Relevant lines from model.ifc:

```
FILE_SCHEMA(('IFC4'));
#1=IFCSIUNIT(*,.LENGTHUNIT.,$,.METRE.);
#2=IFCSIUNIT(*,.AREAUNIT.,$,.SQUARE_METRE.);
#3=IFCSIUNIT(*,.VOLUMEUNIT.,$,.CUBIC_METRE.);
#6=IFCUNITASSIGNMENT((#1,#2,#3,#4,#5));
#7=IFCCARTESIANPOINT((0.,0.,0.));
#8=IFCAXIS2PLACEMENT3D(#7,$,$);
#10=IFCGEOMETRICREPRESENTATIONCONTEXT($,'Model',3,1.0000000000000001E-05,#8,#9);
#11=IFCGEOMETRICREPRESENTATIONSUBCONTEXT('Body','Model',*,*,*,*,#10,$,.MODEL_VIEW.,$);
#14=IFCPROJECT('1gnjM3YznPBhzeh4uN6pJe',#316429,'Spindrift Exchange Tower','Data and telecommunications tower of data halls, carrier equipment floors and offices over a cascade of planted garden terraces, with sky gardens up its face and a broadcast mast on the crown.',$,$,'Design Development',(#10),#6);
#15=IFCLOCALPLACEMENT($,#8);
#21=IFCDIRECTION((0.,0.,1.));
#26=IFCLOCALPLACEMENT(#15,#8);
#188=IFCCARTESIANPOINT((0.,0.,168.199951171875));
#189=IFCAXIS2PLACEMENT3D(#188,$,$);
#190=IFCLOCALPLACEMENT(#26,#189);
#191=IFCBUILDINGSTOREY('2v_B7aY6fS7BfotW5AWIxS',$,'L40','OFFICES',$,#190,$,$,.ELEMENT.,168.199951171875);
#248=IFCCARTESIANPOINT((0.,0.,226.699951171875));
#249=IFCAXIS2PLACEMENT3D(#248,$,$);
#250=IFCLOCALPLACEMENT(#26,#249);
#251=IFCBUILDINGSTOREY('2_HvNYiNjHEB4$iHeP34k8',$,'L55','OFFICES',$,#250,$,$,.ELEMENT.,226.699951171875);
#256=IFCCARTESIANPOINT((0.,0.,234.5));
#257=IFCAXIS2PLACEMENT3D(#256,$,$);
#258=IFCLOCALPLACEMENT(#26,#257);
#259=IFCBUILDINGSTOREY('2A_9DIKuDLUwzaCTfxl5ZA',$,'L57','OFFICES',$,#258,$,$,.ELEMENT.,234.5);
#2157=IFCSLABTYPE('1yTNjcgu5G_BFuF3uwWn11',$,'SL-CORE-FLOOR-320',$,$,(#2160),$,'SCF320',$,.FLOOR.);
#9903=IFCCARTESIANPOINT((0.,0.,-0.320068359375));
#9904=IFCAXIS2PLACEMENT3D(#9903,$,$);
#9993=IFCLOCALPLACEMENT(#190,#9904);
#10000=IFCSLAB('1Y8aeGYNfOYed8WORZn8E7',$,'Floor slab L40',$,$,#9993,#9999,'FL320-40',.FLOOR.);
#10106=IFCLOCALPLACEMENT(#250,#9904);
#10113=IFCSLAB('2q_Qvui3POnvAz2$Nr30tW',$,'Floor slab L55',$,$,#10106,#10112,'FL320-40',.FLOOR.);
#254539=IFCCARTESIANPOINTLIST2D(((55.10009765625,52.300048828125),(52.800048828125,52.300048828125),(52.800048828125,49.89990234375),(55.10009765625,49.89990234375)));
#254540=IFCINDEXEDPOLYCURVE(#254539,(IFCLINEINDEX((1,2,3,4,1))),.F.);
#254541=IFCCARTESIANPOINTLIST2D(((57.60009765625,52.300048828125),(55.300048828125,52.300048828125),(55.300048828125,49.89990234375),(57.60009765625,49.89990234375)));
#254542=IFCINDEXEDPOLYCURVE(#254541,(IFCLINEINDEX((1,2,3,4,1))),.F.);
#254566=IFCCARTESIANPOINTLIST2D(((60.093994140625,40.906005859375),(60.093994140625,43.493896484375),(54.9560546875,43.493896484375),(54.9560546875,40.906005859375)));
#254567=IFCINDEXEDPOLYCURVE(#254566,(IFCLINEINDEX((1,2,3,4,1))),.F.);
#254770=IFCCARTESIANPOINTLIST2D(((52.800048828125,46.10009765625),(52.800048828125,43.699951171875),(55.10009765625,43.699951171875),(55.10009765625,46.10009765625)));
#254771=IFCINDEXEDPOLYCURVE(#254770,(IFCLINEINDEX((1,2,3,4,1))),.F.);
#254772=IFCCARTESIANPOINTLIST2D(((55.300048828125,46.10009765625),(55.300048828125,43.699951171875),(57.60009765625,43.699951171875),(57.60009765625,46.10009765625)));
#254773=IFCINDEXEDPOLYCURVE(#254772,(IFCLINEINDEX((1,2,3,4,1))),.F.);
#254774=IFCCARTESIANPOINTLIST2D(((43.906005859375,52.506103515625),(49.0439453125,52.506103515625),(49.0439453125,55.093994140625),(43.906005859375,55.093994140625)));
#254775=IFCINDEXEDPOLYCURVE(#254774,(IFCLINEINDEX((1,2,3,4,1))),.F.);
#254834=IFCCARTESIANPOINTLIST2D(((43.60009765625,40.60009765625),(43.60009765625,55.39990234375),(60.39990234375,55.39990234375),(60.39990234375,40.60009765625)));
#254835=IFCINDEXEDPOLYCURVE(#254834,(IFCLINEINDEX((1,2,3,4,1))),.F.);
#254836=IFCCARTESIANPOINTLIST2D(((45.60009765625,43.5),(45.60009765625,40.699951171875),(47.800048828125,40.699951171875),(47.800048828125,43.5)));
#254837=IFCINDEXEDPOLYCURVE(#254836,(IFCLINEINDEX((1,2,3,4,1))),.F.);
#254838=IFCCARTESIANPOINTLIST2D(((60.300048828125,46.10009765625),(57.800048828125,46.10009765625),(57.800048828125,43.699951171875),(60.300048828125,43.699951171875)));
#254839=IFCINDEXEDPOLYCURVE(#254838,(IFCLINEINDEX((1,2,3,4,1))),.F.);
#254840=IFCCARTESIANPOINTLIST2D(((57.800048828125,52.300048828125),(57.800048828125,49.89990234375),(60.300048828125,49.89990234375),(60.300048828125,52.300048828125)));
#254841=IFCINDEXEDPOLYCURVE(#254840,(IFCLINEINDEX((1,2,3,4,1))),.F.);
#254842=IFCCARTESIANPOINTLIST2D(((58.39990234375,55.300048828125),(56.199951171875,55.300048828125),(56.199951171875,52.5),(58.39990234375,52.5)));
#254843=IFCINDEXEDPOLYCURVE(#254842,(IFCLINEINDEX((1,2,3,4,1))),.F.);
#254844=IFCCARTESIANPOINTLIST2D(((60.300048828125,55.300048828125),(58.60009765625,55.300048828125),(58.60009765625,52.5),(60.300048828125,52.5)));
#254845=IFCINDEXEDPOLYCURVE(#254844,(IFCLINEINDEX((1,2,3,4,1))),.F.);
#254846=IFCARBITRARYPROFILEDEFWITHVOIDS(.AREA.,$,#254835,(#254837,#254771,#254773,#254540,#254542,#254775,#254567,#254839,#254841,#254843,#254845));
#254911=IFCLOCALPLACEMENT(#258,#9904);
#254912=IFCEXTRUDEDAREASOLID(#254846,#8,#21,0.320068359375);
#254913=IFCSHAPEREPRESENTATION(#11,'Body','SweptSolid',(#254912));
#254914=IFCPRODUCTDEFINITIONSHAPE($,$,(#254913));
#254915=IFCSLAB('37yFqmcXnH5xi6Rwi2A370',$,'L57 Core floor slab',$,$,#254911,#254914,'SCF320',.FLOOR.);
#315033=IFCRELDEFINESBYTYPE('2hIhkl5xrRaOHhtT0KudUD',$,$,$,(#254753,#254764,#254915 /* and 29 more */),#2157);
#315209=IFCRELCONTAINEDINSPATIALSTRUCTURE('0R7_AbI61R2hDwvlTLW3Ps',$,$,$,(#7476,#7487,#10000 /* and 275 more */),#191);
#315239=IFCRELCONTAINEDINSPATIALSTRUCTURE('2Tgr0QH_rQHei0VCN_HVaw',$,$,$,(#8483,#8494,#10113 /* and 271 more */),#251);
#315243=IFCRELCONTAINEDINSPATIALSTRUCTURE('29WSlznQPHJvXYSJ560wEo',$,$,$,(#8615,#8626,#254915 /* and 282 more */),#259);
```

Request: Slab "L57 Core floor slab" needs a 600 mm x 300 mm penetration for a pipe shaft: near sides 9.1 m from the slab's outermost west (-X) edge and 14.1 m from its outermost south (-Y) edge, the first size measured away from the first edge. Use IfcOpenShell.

```python
import numpy as np
import ifcopenshell
import ifcopenshell.api.feature
import ifcopenshell.api.geometry
import ifcopenshell.api.root
import ifcopenshell.geom
import ifcopenshell.util.placement
import ifcopenshell.util.representation
import ifcopenshell.util.shape
import ifcopenshell.util.unit

model = ifcopenshell.open("model.ifc")
unit_scale = ifcopenshell.util.unit.calculate_unit_scale(model)
settings = ifcopenshell.geom.settings()


def volume(element):
    """Net volume in cubic metres, openings subtracted."""
    shape = ifcopenshell.geom.create_shape(settings, element)
    return ifcopenshell.util.shape.get_volume(shape.geometry)


slab = model.by_guid("37yFqmcXnH5xi6Rwi2A370")
before = volume(slab)

# Extent in the slab's own axes, in metres. The edges named are its -X and -Y sides.
slab_shape = ifcopenshell.geom.create_shape(settings, slab)
vertices = ifcopenshell.util.shape.get_vertices(slab_shape.geometry)
x_min, y_min, bottom = vertices.min(axis=0)
top = vertices[:, 2].max()

opening = ifcopenshell.api.root.create_entity(model, ifc_class="IfcOpeningElement", name="Pipe shaft opening", predefined_type="OPENING")
context = ifcopenshell.util.representation.get_context(model, "Model", "Body", "MODEL_VIEW")
width, depth = 0.6, 0.3
outline = [(0.0, 0.0), (width, 0.0), (width, depth), (0.0, depth), (0.0, 0.0)]
# Overshoot both faces by 50 mm so the cut is clean.
shape = ifcopenshell.api.geometry.add_slab_representation(
    model, context=context, depth=top - bottom + 0.1, polyline=outline
)
ifcopenshell.api.geometry.assign_representation(model, product=opening, representation=shape)

matrix = ifcopenshell.util.placement.get_local_placement(slab.ObjectPlacement)
matrix[:, 3] = matrix @ np.append(np.array([x_min + 9.1, y_min + 14.1, bottom - 0.05]) / unit_scale, 1.0)
ifcopenshell.api.geometry.edit_object_placement(model, product=opening, matrix=matrix, is_si=False)
ifcopenshell.api.feature.add_feature(model, feature=opening, element=slab)

after = volume(slab)

print(f"slab volume {before:.3f} -> {after:.3f} m3")

model.write("model_rev.ifc")
```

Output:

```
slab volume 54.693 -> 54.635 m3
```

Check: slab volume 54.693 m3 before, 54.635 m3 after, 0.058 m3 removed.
